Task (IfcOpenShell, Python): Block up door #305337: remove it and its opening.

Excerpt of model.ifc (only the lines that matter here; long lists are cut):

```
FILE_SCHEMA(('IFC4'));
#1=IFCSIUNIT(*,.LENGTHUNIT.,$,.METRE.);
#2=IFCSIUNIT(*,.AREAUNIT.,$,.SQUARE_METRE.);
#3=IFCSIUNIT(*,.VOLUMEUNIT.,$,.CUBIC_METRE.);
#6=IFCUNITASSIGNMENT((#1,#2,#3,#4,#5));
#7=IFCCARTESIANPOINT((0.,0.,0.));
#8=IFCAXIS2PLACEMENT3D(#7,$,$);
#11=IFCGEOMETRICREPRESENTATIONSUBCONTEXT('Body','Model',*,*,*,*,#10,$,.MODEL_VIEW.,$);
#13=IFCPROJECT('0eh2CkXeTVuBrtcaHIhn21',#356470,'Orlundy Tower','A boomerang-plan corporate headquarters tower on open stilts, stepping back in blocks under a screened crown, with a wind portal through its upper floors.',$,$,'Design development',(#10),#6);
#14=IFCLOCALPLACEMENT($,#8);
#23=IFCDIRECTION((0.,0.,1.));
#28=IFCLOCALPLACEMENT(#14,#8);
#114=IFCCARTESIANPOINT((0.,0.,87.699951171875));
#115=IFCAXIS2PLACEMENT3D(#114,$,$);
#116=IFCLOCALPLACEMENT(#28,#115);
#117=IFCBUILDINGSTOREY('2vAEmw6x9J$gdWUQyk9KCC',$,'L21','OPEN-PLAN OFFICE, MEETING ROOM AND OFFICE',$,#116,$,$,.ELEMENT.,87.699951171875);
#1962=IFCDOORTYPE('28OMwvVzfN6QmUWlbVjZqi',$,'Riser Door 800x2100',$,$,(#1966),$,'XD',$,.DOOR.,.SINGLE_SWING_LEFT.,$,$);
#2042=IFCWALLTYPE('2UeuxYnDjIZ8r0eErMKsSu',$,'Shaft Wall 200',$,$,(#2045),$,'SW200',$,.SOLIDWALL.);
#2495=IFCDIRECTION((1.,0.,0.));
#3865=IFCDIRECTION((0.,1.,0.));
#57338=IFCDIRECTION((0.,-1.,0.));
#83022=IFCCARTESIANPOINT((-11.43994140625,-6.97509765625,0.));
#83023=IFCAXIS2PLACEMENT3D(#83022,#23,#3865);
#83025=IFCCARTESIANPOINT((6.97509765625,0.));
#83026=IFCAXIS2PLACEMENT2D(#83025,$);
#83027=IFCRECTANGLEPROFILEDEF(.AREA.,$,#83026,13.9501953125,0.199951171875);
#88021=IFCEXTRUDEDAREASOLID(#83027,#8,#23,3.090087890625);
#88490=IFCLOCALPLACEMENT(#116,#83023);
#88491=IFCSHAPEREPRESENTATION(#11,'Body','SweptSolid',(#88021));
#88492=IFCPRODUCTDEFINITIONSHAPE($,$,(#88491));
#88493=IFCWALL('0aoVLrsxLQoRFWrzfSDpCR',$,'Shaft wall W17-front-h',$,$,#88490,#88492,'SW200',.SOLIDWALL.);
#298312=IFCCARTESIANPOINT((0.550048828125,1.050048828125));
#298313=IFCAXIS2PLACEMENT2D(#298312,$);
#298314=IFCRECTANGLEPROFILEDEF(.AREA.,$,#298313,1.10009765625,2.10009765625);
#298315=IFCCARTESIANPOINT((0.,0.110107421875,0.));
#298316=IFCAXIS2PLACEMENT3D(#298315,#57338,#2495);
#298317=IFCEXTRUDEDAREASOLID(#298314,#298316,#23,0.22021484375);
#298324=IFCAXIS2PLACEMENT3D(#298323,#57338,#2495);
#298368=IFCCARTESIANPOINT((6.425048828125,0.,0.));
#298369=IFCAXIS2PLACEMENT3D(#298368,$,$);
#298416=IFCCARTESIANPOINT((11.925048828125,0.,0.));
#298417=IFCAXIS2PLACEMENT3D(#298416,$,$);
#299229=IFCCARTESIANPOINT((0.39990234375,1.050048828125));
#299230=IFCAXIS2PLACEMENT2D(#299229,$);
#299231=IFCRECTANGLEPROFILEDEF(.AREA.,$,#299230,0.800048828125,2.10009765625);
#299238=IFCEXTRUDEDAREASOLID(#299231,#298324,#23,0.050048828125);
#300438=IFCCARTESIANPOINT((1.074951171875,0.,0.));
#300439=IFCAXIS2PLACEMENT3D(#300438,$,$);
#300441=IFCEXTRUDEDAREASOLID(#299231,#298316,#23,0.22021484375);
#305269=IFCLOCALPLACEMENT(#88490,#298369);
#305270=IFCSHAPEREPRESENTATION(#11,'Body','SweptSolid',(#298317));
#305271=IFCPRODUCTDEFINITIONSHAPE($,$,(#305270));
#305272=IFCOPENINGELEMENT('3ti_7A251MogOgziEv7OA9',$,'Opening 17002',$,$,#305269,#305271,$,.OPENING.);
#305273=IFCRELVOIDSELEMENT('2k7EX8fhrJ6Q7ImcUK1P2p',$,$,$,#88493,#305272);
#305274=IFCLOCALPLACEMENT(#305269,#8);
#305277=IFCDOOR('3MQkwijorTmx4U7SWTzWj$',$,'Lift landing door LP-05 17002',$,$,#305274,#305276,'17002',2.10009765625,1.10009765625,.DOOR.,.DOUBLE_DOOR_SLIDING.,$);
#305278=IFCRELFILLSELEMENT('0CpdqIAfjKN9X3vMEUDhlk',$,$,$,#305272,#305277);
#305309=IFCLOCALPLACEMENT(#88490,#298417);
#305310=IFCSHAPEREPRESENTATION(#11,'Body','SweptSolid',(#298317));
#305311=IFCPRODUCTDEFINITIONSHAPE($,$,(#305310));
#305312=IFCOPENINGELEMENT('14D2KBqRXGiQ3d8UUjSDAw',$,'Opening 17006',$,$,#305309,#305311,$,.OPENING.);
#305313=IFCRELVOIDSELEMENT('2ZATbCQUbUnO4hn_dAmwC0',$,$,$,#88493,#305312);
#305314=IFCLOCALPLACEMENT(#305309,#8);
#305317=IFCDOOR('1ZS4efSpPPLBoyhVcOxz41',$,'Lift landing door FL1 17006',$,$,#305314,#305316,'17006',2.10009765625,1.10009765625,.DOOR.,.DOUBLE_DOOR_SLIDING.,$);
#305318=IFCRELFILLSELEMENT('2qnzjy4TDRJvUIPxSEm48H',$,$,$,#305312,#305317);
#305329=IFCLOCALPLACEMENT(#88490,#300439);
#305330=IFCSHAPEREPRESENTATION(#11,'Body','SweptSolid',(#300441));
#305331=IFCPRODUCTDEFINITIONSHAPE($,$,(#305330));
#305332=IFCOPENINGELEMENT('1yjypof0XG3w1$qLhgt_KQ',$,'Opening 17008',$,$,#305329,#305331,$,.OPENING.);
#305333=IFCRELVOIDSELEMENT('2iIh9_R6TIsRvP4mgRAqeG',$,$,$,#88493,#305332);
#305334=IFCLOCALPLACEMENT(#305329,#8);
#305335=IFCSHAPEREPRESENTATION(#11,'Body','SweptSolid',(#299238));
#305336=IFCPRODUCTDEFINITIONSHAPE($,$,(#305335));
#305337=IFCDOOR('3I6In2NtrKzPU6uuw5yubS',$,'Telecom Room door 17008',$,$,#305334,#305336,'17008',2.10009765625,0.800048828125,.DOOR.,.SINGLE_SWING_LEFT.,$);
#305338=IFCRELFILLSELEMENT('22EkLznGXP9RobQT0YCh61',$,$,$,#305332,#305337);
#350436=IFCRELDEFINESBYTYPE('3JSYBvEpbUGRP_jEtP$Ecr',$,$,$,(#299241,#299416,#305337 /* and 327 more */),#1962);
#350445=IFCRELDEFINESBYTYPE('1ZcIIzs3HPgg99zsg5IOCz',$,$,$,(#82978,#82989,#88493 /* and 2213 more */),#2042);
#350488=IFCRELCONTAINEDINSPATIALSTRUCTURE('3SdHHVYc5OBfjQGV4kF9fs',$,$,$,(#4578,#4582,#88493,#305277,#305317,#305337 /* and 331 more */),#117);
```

```python
import ifcopenshell
import ifcopenshell.api.feature
import ifcopenshell.api.root
import ifcopenshell.geom
import ifcopenshell.util.shape

model = ifcopenshell.open("model.ifc")
settings = ifcopenshell.geom.settings()


def volume(element):
    """Net volume in cubic metres, openings subtracted."""
    shape = ifcopenshell.geom.create_shape(settings, element)
    return ifcopenshell.util.shape.get_volume(shape.geometry)


door = model.by_guid("3I6In2NtrKzPU6uuw5yubS")
opening = door.FillsVoids[0].RelatingOpeningElement
wall = opening.VoidsElements[0].RelatingBuildingElement
before = volume(wall)

ifcopenshell.api.root.remove_product(model, product=door)
ifcopenshell.api.feature.remove_feature(model, feature=opening)

after = volume(wall)

print(f"wall volume {before:.3f} -> {after:.3f} m3")

model.write("model_edited.ifc")
```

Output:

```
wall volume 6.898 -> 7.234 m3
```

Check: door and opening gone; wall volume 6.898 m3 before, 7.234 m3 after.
